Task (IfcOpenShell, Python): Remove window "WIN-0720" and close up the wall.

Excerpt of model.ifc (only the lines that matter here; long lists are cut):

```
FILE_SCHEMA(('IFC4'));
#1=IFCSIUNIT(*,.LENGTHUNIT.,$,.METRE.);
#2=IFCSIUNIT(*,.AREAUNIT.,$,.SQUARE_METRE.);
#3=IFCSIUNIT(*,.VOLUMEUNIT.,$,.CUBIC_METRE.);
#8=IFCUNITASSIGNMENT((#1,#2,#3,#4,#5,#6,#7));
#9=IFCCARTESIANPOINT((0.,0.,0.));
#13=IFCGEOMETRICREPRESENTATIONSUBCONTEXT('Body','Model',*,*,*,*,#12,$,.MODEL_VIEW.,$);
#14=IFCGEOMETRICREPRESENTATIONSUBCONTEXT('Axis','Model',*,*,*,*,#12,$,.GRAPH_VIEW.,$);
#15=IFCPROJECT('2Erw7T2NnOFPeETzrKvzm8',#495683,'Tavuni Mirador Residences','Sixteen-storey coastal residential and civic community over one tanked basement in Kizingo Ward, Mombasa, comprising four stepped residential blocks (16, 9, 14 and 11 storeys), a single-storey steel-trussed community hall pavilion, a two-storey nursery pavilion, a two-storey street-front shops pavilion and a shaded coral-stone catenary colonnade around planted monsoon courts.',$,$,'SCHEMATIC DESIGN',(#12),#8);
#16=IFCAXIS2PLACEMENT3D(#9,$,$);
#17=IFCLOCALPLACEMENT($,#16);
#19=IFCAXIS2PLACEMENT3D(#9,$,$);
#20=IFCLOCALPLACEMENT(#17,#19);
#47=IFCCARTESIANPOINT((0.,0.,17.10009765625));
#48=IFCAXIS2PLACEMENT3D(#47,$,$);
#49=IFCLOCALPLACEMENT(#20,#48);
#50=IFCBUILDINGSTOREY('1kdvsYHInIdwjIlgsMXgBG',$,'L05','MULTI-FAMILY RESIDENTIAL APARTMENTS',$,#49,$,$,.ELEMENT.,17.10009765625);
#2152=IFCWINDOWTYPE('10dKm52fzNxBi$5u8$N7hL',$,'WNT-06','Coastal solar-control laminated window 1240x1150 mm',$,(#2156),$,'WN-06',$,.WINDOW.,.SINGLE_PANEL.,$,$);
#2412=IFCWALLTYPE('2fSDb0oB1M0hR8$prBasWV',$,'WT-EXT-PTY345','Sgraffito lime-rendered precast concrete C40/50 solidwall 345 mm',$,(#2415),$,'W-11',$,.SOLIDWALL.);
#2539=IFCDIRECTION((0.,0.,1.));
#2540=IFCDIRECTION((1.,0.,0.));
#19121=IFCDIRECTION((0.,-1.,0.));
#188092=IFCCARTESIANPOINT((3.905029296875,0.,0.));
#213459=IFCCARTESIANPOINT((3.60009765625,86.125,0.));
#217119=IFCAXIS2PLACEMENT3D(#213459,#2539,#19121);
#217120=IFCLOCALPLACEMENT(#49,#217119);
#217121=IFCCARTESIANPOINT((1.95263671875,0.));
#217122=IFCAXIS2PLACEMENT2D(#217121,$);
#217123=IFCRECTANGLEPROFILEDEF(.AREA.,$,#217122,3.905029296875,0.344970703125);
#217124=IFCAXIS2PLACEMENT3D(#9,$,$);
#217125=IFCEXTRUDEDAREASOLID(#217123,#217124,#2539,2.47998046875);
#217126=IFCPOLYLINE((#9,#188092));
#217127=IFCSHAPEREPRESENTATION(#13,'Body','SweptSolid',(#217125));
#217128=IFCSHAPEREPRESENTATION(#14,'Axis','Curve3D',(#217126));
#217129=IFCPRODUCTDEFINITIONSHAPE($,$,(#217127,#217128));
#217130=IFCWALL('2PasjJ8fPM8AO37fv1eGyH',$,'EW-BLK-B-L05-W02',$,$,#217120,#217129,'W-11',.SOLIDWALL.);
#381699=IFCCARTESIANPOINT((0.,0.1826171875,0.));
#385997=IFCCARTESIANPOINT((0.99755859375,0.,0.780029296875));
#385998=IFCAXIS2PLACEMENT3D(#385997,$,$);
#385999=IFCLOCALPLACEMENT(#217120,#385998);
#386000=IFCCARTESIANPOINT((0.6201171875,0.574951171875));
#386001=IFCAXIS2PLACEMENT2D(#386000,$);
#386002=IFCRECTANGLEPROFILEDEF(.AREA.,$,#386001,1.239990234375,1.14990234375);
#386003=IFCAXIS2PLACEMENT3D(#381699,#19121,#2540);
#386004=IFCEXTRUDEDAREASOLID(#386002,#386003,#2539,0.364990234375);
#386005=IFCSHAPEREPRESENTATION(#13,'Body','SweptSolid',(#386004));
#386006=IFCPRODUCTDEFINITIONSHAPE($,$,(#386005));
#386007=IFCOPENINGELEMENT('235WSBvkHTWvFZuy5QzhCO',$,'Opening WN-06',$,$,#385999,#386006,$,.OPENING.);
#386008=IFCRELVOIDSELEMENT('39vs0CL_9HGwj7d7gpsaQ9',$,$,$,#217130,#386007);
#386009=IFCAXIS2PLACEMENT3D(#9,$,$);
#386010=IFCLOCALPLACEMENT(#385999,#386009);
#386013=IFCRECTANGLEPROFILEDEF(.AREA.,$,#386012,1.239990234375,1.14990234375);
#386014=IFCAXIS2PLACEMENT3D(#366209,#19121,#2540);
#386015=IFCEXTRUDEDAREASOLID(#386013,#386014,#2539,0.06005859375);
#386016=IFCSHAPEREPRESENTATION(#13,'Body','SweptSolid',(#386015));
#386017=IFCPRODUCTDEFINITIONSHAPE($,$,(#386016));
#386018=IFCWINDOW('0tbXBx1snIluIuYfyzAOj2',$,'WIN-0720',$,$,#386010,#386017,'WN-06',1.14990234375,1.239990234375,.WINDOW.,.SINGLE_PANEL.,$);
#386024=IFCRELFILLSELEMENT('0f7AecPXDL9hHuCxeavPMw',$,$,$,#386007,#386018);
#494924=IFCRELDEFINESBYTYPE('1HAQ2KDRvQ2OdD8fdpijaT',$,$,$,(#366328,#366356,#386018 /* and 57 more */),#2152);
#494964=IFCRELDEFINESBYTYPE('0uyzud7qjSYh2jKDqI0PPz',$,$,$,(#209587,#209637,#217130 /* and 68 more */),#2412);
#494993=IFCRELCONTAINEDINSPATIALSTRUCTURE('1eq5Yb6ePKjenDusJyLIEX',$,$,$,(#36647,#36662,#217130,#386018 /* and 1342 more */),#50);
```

```python
import ifcopenshell
import ifcopenshell.api.feature
import ifcopenshell.api.root
import ifcopenshell.geom
import ifcopenshell.util.shape

model = ifcopenshell.open("model.ifc")
settings = ifcopenshell.geom.settings()


def volume(element):
    """Net volume in cubic metres, openings subtracted."""
    shape = ifcopenshell.geom.create_shape(settings, element)
    return ifcopenshell.util.shape.get_volume(shape.geometry)


window = model.by_guid("0tbXBx1snIluIuYfyzAOj2")
opening = window.FillsVoids[0].RelatingOpeningElement
wall = opening.VoidsElements[0].RelatingBuildingElement
before = volume(wall)

ifcopenshell.api.root.remove_product(model, product=window)
ifcopenshell.api.feature.remove_feature(model, feature=opening)

after = volume(wall)

print(f"wall volume {before:.3f} -> {after:.3f} m3")

model.write("model_edited.ifc")
```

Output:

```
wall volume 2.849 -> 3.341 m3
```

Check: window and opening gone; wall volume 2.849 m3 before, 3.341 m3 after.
